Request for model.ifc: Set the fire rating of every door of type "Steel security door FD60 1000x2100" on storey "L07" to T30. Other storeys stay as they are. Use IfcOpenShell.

First a look at what the model holds.

```python
import ifcopenshell
import ifcopenshell.util.element

model = ifcopenshell.open("model.ifc")
print(model.schema)
storey = next(s for s in model.by_type("IfcBuildingStorey") if s.Name == "L07")
doors = [e for e in ifcopenshell.util.element.get_decomposition(storey) if e.is_a("IfcDoor")]
seen = {}
for e in doors:
    element_type = ifcopenshell.util.element.get_type(e)
    key = (element_type.Name if element_type != e and element_type else None, ifcopenshell.util.element.get_pset(e, "Pset_DoorCommon", "FireRating"))
    seen[key] = seen.get(key, 0) + 1
for (name, value), count in sorted(seen.items(), key=str):
    print(count, "x", name, "|", value)
```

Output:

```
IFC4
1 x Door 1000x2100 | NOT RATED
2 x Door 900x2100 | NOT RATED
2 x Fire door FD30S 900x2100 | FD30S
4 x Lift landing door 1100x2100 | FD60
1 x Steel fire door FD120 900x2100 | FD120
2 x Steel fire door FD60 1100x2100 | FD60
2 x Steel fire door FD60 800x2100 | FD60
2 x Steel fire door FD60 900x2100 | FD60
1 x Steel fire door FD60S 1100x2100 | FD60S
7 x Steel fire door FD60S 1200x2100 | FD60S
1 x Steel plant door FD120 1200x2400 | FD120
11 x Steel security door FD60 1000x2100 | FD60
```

```python
import ifcopenshell
import ifcopenshell.api.pset
import ifcopenshell.util.element

model = ifcopenshell.open("model.ifc")

storey = next(s for s in model.by_type("IfcBuildingStorey") if s.Name == "L07")
doors = [e for e in ifcopenshell.util.element.get_decomposition(storey) if e.is_a("IfcDoor")]

count = 0
for e in doors:
    element_type = ifcopenshell.util.element.get_type(e)
    if element_type in (None, e) or element_type.Name != "Steel security door FD60 1000x2100":
        continue
    # add_pset returns the element's existing set when there is one.
    pset = ifcopenshell.api.pset.add_pset(model, product=e, name="Pset_DoorCommon")
    ifcopenshell.api.pset.edit_pset(model, pset=pset, properties={"FireRating": "T30"})
    count += 1

print(count, "doors updated")

model.write("model-out.ifc")
```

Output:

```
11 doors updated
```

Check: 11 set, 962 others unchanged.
